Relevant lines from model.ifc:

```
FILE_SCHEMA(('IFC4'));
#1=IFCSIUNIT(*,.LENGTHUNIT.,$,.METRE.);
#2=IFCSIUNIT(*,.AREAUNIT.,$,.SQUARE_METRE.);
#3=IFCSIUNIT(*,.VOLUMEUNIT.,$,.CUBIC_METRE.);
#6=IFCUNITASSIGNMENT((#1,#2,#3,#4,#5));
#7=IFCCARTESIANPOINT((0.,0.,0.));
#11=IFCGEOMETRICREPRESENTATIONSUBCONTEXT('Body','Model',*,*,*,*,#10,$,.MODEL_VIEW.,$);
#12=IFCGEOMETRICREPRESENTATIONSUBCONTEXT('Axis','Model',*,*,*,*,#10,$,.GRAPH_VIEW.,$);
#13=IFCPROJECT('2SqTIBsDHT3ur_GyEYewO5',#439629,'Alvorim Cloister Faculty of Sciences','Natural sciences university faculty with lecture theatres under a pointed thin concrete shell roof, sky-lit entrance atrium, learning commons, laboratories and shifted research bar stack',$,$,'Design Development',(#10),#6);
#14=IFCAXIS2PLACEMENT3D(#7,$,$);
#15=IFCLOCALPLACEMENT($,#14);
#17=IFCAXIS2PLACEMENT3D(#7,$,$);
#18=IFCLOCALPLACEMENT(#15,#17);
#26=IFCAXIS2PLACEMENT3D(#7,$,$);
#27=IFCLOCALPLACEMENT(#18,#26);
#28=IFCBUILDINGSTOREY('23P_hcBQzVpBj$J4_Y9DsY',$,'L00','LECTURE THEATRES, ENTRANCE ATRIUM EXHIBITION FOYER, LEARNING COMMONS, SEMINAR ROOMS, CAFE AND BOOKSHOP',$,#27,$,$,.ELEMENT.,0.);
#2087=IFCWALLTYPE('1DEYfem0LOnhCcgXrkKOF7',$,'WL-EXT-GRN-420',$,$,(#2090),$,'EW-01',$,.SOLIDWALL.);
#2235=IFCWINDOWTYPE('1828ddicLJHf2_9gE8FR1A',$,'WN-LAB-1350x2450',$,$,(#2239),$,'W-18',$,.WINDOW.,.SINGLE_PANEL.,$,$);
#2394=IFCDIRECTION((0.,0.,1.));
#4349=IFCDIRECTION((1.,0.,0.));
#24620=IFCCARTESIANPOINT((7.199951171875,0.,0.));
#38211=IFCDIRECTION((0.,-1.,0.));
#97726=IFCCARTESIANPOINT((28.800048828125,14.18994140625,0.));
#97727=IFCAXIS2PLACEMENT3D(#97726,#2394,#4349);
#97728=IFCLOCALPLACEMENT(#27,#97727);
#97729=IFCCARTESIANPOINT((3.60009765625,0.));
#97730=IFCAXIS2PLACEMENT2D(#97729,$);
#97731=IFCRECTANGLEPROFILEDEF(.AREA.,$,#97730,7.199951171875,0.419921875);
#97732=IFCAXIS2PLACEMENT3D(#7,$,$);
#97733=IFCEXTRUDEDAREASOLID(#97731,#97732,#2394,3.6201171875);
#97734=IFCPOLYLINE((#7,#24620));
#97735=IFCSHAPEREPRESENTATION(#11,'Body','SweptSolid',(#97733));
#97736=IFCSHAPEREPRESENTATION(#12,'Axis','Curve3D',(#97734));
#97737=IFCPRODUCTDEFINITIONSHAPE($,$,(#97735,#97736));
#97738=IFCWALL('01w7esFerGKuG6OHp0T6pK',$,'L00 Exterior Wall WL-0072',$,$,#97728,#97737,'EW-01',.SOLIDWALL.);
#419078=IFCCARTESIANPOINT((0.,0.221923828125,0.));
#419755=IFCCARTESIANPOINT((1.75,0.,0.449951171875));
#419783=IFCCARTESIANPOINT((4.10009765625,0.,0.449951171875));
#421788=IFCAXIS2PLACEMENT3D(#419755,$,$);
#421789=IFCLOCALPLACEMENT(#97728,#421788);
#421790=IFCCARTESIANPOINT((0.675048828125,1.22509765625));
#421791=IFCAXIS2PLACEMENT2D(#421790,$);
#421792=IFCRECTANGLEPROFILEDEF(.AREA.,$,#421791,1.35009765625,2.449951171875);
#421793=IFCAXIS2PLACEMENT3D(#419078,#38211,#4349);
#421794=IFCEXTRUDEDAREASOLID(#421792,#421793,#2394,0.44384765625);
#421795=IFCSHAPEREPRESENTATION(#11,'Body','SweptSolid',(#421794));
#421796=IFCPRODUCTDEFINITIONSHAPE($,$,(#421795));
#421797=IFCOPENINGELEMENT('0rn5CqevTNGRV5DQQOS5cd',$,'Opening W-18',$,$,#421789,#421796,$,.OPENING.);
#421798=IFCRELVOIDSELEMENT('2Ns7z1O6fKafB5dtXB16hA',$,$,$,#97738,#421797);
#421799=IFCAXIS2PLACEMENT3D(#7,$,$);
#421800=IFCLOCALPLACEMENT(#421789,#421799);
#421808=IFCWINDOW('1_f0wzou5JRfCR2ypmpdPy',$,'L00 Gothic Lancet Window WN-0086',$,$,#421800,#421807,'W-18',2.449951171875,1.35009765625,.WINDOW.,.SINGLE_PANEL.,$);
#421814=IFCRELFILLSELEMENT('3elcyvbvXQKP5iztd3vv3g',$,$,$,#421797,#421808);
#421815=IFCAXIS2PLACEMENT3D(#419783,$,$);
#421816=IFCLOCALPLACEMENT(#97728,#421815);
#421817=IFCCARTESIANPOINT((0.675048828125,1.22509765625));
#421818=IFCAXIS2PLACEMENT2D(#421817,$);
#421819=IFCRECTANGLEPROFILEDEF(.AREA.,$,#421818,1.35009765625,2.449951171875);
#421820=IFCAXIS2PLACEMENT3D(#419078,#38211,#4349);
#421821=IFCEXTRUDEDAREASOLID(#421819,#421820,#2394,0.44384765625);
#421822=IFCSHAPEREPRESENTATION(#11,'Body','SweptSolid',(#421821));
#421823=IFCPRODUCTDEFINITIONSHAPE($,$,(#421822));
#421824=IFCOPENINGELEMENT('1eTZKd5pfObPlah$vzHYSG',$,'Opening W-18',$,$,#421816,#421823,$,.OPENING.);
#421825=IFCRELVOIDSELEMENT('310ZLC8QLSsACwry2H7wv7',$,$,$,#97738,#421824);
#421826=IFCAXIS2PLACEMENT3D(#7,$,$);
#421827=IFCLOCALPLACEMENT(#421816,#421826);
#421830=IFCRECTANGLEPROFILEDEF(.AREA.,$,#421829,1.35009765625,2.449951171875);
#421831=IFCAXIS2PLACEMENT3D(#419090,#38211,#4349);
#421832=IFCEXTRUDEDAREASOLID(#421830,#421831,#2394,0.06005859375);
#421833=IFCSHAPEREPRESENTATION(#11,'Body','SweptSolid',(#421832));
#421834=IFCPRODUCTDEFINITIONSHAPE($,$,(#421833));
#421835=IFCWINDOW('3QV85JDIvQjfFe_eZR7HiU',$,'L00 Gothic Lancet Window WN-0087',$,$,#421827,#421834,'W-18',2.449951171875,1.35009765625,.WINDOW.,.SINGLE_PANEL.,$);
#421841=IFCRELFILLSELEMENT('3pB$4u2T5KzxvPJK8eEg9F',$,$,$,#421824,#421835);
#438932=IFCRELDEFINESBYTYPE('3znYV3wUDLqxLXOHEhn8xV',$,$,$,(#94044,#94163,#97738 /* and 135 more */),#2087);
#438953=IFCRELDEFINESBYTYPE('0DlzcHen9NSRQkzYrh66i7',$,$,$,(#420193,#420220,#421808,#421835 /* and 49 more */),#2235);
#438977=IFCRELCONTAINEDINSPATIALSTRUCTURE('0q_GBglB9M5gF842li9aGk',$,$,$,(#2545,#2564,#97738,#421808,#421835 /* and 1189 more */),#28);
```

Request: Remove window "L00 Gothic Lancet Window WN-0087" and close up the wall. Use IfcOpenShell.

```python
import ifcopenshell
import ifcopenshell.api.feature
import ifcopenshell.api.root
import ifcopenshell.geom
import ifcopenshell.util.shape

model = ifcopenshell.open("model.ifc")
settings = ifcopenshell.geom.settings()


def volume(element):
    """Net volume in cubic metres, openings subtracted."""
    shape = ifcopenshell.geom.create_shape(settings, element)
    return ifcopenshell.util.shape.get_volume(shape.geometry)


window = model.by_id(421835)
opening = window.FillsVoids[0].RelatingOpeningElement
wall = opening.VoidsElements[0].RelatingBuildingElement
before = volume(wall)

ifcopenshell.api.root.remove_product(model, product=window)
ifcopenshell.api.feature.remove_feature(model, feature=opening)

after = volume(wall)

print(f"wall volume {before:.3f} -> {after:.3f} m3")

model.write("model_rev.ifc")
```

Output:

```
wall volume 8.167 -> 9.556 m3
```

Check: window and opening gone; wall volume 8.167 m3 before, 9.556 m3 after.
